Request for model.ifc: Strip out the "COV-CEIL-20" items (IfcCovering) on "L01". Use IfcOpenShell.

First a look at what the model holds.

```python
import ifcopenshell
import ifcopenshell.util.element

model = ifcopenshell.open("model.ifc")
print(model.schema)
storey = next(s for s in model.by_type("IfcBuildingStorey") if s.Name == "L01")
coverings = [e for e in ifcopenshell.util.element.get_decomposition(storey) if e.is_a("IfcCovering")]
seen = {}
for e in coverings:
    element_type = ifcopenshell.util.element.get_type(e)
    name = element_type.Name if element_type not in (None, e) else None
    seen[name] = seen.get(name, 0) + 1
for name, count in sorted(seen.items(), key=str):
    print(count, "x", name)
```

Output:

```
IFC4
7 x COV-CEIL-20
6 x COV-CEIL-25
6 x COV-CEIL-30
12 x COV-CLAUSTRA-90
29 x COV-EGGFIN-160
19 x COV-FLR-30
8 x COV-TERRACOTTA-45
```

```python
import ifcopenshell
import ifcopenshell.api.root
import ifcopenshell.util.element

model = ifcopenshell.open("model.ifc")

storey = next(s for s in model.by_type("IfcBuildingStorey") if s.Name == "L01")
coverings = [e for e in ifcopenshell.util.element.get_decomposition(storey) if e.is_a("IfcCovering")]
targets = [e for e in coverings if (t := ifcopenshell.util.element.get_type(e)) not in (None, e) and t.Name == "COV-CEIL-20"]

for e in targets:
    ifcopenshell.api.root.remove_product(model, product=e)
print(len(targets), "removed")

model.write("model_edited.ifc")
```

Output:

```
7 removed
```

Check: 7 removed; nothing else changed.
